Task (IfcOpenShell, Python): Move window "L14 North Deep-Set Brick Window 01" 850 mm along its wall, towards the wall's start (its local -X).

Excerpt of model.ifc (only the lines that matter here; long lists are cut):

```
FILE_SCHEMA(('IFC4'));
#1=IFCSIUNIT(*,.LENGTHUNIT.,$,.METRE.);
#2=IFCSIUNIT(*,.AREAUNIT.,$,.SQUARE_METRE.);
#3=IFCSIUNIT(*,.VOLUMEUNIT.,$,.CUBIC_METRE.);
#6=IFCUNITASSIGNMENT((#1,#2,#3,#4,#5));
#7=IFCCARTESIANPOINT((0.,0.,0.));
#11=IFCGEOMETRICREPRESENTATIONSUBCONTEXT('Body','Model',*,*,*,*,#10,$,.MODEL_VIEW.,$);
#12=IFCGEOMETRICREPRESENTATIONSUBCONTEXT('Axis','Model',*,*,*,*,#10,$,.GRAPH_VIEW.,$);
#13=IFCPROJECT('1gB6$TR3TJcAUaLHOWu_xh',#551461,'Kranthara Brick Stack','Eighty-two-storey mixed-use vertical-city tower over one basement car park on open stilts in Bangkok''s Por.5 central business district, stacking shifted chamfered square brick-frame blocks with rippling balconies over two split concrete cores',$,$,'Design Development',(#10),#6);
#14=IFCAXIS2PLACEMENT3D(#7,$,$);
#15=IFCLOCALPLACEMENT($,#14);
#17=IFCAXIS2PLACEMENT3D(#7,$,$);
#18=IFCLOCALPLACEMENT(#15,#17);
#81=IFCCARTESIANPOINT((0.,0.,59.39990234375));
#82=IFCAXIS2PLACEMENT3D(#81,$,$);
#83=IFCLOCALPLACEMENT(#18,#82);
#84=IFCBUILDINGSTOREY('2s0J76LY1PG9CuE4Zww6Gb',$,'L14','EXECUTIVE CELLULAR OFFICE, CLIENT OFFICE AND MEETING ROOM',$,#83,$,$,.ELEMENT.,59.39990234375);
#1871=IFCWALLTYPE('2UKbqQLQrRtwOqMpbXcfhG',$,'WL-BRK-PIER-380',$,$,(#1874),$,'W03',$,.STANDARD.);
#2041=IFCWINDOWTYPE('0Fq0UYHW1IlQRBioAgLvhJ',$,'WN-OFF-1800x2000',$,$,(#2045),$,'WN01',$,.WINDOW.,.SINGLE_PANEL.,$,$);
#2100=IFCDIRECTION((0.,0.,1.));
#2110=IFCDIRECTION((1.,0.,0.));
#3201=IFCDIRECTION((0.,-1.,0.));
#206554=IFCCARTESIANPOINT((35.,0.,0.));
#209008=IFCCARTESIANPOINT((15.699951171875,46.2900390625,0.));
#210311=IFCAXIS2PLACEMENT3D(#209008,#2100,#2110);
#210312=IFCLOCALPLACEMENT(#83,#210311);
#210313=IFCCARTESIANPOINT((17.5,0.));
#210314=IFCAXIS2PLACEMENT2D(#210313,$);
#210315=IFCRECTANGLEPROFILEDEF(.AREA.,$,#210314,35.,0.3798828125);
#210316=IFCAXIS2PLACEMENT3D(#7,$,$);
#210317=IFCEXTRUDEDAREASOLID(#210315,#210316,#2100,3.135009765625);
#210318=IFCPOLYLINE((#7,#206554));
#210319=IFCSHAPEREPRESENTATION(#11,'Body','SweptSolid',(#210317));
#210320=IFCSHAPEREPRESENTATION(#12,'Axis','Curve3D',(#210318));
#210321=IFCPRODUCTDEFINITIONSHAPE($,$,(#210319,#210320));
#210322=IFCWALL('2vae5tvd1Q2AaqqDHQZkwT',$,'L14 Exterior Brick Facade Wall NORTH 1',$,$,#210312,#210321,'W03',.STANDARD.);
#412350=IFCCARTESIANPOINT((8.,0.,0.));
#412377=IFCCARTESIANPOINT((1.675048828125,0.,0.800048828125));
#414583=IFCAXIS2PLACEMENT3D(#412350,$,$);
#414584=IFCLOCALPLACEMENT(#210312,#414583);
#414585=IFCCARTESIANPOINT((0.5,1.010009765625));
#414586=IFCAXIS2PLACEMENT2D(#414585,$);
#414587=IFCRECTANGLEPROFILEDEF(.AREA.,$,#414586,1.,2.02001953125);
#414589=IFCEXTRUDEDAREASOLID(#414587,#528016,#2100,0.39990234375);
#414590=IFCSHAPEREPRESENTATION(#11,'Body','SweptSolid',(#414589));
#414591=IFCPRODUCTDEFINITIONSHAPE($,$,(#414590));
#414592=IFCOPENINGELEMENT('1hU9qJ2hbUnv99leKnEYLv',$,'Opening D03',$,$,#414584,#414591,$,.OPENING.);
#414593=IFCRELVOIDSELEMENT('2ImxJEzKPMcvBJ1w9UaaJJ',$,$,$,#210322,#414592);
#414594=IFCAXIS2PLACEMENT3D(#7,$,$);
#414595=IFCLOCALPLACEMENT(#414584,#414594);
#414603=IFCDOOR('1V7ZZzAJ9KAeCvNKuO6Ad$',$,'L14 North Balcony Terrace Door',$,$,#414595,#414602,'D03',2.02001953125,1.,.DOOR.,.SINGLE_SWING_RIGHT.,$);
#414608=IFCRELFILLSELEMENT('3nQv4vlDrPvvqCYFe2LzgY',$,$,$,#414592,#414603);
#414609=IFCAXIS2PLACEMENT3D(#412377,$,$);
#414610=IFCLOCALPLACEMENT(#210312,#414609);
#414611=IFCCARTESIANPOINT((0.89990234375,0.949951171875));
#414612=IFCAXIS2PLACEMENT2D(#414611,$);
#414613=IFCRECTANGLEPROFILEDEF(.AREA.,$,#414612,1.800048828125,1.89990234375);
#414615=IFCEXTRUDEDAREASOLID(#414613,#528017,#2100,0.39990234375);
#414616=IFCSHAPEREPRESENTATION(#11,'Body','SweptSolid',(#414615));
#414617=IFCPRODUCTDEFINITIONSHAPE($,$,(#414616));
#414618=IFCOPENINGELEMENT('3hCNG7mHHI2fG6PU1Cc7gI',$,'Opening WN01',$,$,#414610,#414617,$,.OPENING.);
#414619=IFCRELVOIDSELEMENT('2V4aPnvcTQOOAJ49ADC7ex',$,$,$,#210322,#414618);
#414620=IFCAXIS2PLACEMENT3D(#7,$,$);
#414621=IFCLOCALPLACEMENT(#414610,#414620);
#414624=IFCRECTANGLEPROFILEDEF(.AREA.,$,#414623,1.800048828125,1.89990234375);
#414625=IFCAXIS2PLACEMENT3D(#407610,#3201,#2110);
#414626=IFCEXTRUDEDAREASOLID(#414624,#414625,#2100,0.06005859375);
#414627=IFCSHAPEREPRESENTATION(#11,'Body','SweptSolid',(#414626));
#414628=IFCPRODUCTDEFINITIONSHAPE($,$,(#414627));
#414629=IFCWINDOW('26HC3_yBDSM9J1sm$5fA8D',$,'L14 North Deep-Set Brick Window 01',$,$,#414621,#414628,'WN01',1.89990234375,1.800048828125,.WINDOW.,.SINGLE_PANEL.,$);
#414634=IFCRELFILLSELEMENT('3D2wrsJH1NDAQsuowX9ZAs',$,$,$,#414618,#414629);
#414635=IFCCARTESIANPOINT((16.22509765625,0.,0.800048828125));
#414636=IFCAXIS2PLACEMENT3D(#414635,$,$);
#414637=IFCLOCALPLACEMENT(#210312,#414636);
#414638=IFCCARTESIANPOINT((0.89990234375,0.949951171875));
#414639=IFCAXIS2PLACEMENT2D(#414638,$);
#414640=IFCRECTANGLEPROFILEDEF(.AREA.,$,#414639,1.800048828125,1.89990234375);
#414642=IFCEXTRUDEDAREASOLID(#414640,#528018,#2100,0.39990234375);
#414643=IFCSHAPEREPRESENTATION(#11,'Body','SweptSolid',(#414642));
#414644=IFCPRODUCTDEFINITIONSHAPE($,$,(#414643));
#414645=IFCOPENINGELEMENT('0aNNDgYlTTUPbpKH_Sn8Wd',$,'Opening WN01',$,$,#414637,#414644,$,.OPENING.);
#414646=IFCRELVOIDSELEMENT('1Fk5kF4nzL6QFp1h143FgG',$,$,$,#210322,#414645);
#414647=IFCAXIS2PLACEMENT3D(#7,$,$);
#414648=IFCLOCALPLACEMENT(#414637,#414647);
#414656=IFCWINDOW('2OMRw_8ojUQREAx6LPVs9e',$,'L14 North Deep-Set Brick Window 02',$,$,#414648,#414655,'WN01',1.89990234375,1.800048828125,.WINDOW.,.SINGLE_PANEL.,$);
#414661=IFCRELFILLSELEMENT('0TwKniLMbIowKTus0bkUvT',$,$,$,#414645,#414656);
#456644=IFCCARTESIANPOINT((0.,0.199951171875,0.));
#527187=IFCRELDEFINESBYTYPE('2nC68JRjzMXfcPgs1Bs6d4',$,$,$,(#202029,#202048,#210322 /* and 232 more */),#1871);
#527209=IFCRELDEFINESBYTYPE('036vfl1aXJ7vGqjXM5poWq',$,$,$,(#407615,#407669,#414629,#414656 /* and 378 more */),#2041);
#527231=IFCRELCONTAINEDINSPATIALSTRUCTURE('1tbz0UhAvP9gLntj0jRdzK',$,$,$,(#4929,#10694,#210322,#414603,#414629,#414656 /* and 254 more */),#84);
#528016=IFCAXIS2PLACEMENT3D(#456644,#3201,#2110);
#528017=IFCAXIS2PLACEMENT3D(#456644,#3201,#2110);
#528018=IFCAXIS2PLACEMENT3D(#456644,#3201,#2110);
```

```python
import ifcopenshell
import ifcopenshell.api.geometry
import ifcopenshell.util.placement
import ifcopenshell.util.unit

model = ifcopenshell.open("model.ifc")
unit_scale = ifcopenshell.util.unit.calculate_unit_scale(model)

window = model.by_guid("26HC3_yBDSM9J1sm$5fA8D")
opening = window.FillsVoids[0].RelatingOpeningElement
wall = opening.VoidsElements[0].RelatingBuildingElement

wall_matrix = ifcopenshell.util.placement.get_local_placement(wall.ObjectPlacement)
shift = wall_matrix[:3, 0] * -0.85 / unit_scale
before = ifcopenshell.util.placement.get_local_placement(window.ObjectPlacement)[:3, 3].copy()

# The window is placed relative to its opening, so it follows when the opening moves.
matrix = ifcopenshell.util.placement.get_local_placement(opening.ObjectPlacement)
matrix[:3, 3] += shift
ifcopenshell.api.geometry.edit_object_placement(
    model, product=opening, matrix=matrix, is_si=False, should_transform_children=True
)

after = ifcopenshell.util.placement.get_local_placement(window.ObjectPlacement)[:3, 3]
print("window moved by", (after - before).round(3) + 0.0)

model.write("model-out.ifc")
```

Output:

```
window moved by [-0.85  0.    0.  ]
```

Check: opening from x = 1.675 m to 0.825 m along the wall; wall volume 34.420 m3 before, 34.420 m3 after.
